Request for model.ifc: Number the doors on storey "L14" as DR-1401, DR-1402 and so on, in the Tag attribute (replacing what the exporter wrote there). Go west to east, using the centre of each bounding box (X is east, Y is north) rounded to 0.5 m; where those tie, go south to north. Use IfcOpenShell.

First a look at what the model holds.

```python
import ifcopenshell
import ifcopenshell.util.element
import ifcopenshell.util.placement

model = ifcopenshell.open("model.ifc")
print(model.schema)
storey = next(s for s in model.by_type("IfcBuildingStorey") if s.Name == "L14")
doors = [e for e in ifcopenshell.util.element.get_decomposition(storey) if e.is_a("IfcDoor")]
for e in sorted(doors, key=lambda e: e.id()):
    origin = ifcopenshell.util.placement.get_local_placement(e.ObjectPlacement)[:3, 3]
    print(e.id(), e.Tag, e.Name, origin.round(2) + 0.0, sep=" | ")
```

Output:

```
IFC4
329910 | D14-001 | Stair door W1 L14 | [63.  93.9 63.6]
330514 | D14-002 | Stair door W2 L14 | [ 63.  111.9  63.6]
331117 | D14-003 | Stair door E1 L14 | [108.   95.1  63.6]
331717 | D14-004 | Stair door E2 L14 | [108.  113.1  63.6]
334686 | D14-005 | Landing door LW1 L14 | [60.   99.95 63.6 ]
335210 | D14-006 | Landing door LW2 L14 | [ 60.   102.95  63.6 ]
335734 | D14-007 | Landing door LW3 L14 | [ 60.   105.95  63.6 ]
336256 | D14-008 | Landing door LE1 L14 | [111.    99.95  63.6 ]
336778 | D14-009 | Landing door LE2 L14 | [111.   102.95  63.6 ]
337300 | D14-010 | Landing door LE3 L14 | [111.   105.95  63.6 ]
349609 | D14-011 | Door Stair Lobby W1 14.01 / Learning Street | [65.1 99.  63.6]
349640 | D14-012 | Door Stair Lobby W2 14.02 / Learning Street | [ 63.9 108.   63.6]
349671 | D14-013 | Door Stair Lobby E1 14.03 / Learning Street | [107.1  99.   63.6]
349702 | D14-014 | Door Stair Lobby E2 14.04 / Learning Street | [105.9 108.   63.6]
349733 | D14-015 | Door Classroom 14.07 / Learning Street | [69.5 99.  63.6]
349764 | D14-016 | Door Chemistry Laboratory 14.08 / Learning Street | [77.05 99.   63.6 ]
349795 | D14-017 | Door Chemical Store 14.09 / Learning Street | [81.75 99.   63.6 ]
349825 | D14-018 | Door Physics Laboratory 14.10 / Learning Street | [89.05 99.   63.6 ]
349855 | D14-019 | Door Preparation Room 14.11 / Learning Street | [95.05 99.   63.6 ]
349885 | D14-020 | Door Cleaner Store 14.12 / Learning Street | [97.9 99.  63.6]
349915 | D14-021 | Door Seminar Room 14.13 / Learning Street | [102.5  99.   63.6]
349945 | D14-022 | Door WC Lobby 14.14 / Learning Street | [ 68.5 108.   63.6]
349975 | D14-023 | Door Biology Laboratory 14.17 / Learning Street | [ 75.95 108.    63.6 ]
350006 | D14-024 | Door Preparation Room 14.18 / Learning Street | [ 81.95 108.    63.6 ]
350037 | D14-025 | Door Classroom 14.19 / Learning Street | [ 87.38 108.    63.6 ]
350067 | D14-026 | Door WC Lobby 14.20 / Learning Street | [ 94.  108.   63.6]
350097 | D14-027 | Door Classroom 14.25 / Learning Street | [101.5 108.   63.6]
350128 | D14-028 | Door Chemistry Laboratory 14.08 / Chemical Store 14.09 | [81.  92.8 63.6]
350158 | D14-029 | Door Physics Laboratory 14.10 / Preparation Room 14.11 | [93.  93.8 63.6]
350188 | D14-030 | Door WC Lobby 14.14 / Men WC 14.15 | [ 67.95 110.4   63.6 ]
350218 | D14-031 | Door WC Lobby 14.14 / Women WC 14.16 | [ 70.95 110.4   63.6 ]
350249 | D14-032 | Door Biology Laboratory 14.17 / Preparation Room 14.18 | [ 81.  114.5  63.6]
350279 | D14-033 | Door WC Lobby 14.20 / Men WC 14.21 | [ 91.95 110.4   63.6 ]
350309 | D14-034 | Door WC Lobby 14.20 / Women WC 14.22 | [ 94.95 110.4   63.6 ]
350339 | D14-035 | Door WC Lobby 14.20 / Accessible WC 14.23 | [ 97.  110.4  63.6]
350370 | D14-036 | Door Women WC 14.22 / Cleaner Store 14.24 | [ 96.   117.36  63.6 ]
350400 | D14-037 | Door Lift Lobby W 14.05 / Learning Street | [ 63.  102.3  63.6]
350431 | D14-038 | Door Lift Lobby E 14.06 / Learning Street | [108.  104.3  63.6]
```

```python
import ifcopenshell
import ifcopenshell.geom
import ifcopenshell.util.element
import ifcopenshell.util.shape

model = ifcopenshell.open("model.ifc")
settings = ifcopenshell.geom.settings()
settings.set("use-world-coords", True)


def centre(element):
    shape = ifcopenshell.geom.create_shape(settings, element)
    return ifcopenshell.util.shape.get_bbox_centroid(shape.geometry)


storey = next(s for s in model.by_type("IfcBuildingStorey") if s.Name == "L14")
doors = [e for e in ifcopenshell.util.element.get_decomposition(storey) if e.is_a("IfcDoor")]

# Insertion points can sit at a corner or the storey origin, so sort by the geometry (in metres).
centres = {e: centre(e) for e in doors}
doors.sort(key=lambda e: (round(centres[e][0] / 0.5), centres[e][1]))

for i, e in enumerate(doors, start=1):
    number = f"DR-14{i:02d}"
    e.Tag = number
    print(e.id(), number)

model.write("model_v2.ifc")
```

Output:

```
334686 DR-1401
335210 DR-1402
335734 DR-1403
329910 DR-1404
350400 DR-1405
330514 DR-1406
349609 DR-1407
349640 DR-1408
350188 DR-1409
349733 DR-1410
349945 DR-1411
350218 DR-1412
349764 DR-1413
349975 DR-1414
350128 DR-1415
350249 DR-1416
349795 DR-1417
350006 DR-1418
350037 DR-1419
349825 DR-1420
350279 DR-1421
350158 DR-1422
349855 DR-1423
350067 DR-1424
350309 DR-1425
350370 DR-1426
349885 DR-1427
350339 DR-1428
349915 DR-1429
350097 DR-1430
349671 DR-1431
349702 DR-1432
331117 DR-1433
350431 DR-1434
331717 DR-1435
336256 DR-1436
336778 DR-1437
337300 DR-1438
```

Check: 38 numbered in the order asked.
